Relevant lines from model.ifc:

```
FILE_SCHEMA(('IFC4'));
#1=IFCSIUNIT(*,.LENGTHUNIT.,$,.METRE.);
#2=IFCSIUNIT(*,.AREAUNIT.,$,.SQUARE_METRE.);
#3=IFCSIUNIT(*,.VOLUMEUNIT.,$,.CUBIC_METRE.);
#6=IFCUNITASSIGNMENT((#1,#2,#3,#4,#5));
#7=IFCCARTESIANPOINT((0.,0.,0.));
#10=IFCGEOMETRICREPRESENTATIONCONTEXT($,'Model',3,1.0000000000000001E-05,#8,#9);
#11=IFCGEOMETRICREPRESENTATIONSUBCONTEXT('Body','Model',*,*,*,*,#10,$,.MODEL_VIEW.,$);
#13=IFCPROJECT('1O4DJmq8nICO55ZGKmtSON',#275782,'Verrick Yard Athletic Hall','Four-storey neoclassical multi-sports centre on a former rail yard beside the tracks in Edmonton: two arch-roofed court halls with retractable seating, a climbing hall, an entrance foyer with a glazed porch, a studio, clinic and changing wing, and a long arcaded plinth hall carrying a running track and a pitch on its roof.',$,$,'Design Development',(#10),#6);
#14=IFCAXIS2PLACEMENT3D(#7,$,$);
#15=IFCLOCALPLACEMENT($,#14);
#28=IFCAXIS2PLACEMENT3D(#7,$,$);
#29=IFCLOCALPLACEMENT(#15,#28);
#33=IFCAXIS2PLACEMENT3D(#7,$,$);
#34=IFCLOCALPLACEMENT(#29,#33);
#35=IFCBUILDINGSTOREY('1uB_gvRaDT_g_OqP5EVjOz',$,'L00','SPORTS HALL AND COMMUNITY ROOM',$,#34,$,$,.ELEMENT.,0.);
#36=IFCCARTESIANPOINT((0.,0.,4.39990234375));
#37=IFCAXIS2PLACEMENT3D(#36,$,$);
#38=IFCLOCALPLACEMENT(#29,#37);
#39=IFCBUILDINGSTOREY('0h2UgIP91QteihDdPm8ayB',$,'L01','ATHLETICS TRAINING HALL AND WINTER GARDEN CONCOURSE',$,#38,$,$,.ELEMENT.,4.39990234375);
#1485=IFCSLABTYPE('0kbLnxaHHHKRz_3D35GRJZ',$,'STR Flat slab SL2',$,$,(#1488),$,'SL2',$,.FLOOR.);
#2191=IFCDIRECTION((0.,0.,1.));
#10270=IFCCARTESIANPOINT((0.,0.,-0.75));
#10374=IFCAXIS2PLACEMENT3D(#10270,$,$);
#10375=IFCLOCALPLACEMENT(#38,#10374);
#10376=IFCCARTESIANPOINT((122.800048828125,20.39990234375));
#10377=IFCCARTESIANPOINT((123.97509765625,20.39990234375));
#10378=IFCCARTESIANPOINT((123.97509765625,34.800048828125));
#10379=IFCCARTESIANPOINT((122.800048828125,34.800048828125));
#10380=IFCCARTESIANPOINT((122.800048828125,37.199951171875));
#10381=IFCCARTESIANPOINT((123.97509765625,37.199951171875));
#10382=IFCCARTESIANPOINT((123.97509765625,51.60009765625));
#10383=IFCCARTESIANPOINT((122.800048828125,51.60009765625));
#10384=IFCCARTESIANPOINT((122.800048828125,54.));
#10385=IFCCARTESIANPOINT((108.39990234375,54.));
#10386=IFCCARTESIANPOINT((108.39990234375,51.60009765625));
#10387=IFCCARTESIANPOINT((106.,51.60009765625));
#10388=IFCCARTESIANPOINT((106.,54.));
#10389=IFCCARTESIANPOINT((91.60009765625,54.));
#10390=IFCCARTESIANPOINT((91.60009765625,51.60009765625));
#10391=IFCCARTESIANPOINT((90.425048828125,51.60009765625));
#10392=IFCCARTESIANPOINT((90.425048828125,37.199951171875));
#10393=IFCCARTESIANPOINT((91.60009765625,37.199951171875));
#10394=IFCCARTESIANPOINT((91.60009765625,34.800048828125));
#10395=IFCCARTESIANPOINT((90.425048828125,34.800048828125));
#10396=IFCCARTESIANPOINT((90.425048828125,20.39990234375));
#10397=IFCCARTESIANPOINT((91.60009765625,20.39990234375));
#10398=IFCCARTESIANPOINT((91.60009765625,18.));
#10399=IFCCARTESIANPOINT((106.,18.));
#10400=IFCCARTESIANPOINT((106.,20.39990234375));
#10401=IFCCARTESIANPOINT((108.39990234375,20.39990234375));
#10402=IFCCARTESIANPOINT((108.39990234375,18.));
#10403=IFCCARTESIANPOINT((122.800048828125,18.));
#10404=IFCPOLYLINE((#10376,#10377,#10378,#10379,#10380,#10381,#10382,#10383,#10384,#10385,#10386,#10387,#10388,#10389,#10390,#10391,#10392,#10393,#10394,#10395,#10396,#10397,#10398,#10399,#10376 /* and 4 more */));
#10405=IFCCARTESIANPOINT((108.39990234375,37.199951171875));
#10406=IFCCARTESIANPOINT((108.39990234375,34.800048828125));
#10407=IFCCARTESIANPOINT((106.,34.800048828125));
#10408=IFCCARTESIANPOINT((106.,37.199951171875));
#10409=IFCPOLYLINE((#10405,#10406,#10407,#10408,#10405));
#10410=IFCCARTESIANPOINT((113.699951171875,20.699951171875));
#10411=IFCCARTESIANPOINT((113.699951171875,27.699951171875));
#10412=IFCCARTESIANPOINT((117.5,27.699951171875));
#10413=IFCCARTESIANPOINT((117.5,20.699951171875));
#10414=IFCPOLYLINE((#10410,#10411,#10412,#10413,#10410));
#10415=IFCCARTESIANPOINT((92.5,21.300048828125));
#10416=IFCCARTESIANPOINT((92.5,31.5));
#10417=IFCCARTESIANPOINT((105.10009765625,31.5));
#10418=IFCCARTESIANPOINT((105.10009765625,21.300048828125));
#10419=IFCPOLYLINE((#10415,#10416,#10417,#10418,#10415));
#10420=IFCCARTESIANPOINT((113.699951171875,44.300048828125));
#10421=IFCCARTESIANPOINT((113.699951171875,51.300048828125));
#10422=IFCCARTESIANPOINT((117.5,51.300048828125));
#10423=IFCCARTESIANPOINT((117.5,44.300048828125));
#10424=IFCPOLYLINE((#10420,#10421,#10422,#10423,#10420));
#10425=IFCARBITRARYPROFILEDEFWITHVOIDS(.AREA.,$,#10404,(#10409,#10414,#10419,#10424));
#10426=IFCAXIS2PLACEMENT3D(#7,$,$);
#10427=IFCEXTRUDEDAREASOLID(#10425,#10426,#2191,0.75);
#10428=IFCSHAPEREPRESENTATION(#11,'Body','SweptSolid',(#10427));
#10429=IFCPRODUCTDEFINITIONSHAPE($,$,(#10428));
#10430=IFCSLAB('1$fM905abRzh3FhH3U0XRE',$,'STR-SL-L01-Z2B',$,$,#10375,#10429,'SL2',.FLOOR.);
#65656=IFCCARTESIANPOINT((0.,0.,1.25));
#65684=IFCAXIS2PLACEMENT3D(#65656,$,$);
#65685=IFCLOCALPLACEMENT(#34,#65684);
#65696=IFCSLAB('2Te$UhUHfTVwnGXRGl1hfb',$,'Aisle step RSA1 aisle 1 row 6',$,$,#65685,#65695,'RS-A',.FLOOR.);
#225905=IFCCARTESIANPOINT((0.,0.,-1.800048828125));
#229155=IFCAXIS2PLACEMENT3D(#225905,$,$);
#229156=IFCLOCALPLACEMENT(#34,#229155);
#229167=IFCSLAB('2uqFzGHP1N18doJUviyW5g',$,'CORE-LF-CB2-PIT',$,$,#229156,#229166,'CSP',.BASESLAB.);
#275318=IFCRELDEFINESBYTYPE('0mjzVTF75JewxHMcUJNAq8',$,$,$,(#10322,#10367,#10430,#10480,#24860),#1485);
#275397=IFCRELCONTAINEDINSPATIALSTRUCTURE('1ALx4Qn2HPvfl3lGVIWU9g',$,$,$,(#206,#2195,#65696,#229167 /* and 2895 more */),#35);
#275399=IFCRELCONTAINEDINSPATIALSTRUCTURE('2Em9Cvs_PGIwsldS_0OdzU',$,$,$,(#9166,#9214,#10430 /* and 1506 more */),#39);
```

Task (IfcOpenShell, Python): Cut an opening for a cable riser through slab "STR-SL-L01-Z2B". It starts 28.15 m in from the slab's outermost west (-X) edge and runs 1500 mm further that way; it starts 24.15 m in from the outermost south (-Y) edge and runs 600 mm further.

```python
import numpy as np
import ifcopenshell
import ifcopenshell.api.feature
import ifcopenshell.api.geometry
import ifcopenshell.api.root
import ifcopenshell.geom
import ifcopenshell.util.placement
import ifcopenshell.util.representation
import ifcopenshell.util.shape
import ifcopenshell.util.unit

model = ifcopenshell.open("model.ifc")
unit_scale = ifcopenshell.util.unit.calculate_unit_scale(model)
settings = ifcopenshell.geom.settings()


def volume(element):
    """Net volume in cubic metres, openings subtracted."""
    shape = ifcopenshell.geom.create_shape(settings, element)
    return ifcopenshell.util.shape.get_volume(shape.geometry)


slab = model.by_guid("1$fM905abRzh3FhH3U0XRE")
before = volume(slab)

# Extent in the slab's own axes, in metres. The edges named are its -X and -Y sides.
slab_shape = ifcopenshell.geom.create_shape(settings, slab)
vertices = ifcopenshell.util.shape.get_vertices(slab_shape.geometry)
x_min, y_min, bottom = vertices.min(axis=0)
top = vertices[:, 2].max()

opening = ifcopenshell.api.root.create_entity(model, ifc_class="IfcOpeningElement", name="Cable riser opening", predefined_type="OPENING")
context = ifcopenshell.util.representation.get_context(model, "Model", "Body", "MODEL_VIEW")
width, depth = 1.5, 0.6
outline = [(0.0, 0.0), (width, 0.0), (width, depth), (0.0, depth), (0.0, 0.0)]
# Overshoot both faces by 50 mm so the cut is clean.
shape = ifcopenshell.api.geometry.add_slab_representation(
    model, context=context, depth=top - bottom + 0.1, polyline=outline
)
ifcopenshell.api.geometry.assign_representation(model, product=opening, representation=shape)

matrix = ifcopenshell.util.placement.get_local_placement(slab.ObjectPlacement)
matrix[:, 3] = matrix @ np.append(np.array([x_min + 28.15, y_min + 24.15, bottom - 0.05]) / unit_scale, 1.0)
ifcopenshell.api.geometry.edit_object_placement(model, product=opening, matrix=matrix, is_si=False)
ifcopenshell.api.feature.add_feature(model, feature=opening, element=slab)

after = volume(slab)

print(f"slab volume {before:.3f} -> {after:.3f} m3")

model.write("model_rev.ifc")
```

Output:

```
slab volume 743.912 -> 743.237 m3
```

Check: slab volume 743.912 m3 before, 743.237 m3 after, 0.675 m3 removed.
